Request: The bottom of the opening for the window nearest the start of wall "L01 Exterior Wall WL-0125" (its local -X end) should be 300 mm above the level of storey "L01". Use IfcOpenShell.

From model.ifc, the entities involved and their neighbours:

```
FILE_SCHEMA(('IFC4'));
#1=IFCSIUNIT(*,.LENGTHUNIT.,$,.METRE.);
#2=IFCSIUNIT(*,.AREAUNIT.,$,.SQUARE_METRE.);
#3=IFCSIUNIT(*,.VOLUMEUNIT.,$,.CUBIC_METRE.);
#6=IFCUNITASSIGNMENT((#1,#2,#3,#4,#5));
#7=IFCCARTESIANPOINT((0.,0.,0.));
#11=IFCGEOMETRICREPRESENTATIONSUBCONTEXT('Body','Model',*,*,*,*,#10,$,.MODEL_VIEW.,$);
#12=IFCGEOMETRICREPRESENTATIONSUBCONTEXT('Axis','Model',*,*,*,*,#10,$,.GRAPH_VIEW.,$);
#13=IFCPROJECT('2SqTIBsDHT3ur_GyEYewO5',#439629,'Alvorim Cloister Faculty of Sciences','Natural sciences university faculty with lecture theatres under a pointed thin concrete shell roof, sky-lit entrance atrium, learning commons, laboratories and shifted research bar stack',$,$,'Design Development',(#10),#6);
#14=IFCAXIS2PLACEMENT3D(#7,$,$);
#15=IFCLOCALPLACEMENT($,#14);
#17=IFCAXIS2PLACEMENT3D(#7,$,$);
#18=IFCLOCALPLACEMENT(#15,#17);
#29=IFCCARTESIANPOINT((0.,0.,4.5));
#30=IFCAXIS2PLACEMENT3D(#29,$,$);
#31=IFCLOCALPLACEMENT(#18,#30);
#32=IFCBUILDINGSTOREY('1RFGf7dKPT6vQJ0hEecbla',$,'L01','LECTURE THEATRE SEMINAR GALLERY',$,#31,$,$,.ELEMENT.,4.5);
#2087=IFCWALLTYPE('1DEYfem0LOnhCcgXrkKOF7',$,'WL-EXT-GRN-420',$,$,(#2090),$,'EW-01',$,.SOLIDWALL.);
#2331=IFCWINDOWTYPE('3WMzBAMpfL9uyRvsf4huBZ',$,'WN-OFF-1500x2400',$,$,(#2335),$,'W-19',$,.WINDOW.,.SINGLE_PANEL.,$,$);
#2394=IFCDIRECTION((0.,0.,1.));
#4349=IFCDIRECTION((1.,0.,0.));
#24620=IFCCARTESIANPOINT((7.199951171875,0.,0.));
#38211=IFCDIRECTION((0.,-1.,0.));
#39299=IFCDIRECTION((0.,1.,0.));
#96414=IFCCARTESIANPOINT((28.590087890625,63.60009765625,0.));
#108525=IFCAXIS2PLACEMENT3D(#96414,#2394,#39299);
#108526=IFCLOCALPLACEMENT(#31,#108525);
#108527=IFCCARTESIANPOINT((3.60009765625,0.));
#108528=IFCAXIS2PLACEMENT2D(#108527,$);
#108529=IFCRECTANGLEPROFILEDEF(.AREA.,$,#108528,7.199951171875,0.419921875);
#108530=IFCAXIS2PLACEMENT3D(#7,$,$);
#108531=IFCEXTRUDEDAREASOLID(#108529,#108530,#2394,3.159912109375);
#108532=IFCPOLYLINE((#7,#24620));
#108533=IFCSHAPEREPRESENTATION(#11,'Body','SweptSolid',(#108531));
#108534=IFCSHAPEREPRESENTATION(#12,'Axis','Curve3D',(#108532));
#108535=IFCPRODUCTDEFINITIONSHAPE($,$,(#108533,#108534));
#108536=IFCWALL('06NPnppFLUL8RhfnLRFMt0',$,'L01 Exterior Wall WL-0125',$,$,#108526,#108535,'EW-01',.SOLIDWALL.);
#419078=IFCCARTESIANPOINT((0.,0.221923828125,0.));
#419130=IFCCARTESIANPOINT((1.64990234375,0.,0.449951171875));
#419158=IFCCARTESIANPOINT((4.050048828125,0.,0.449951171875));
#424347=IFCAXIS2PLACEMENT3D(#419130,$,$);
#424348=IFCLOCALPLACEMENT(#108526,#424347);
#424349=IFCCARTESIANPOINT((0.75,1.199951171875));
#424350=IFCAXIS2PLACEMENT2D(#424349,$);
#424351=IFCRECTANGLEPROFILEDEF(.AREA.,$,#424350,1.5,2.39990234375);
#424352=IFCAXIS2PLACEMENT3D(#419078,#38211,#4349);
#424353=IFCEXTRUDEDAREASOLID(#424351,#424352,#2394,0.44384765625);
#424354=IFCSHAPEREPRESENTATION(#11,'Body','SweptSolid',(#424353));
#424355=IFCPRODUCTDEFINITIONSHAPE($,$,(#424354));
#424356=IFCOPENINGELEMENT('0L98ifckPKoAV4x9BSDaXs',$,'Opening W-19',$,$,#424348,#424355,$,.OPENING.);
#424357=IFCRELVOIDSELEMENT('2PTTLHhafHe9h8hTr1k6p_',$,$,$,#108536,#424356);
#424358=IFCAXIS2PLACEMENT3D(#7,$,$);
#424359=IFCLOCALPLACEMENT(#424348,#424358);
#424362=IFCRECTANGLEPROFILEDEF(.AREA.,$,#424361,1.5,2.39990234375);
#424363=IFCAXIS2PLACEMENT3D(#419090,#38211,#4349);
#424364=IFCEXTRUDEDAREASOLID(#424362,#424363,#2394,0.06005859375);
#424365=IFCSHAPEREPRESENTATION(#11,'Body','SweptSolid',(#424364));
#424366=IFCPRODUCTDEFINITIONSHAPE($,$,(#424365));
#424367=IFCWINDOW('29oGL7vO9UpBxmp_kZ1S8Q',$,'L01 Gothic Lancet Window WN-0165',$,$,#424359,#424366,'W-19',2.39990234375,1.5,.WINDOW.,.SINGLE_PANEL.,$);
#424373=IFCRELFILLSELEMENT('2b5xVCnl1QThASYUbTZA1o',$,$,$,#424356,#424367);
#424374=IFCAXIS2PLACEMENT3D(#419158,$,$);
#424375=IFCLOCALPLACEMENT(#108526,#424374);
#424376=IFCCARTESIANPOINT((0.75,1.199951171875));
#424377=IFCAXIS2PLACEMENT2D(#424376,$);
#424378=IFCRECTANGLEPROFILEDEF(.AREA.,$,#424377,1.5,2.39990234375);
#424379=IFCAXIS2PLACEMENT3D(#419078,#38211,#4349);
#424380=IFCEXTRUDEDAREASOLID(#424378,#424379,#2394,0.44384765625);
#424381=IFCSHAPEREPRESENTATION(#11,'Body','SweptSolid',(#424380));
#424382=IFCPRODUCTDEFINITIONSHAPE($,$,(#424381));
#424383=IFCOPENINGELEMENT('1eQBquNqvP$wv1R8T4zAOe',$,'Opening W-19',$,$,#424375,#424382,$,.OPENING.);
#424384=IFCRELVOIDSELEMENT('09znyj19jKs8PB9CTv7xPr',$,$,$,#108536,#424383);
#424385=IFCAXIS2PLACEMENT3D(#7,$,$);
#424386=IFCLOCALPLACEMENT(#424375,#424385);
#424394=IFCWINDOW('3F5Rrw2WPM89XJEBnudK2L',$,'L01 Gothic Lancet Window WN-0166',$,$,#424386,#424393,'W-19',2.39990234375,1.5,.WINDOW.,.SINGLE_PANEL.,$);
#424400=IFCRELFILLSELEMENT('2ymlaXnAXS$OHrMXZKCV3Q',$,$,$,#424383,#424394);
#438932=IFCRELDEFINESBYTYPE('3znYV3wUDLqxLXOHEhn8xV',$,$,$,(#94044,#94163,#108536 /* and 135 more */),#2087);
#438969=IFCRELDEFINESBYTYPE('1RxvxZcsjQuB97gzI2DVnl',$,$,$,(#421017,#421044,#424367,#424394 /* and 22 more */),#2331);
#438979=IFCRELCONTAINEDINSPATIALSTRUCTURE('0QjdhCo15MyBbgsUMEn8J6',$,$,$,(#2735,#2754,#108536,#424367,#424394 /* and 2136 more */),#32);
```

```python
import numpy as np
import ifcopenshell
import ifcopenshell.api.geometry
import ifcopenshell.geom
import ifcopenshell.util.element
import ifcopenshell.util.placement
import ifcopenshell.util.shape
import ifcopenshell.util.unit

model = ifcopenshell.open("model.ifc")
unit_scale = ifcopenshell.util.unit.calculate_unit_scale(model)

window = model.by_guid("29oGL7vO9UpBxmp_kZ1S8Q")
opening = window.FillsVoids[0].RelatingOpeningElement
storey = ifcopenshell.util.element.get_container(window, ifc_class="IfcBuildingStorey")
level = ifcopenshell.util.placement.get_local_placement(storey.ObjectPlacement)[2, 3]

# The opening's origin need not be at the sill, so measure its lowest point.
shape = ifcopenshell.geom.create_shape(ifcopenshell.geom.settings(), opening)
bottom = ifcopenshell.util.shape.get_shape_bottom_elevation(shape, shape.geometry) / unit_scale
dz = level + 0.3 / unit_scale - bottom

shift = np.array([0.0, 0.0, dz])
# The window is placed relative to its opening, so it follows when the opening moves.
matrix = ifcopenshell.util.placement.get_local_placement(opening.ObjectPlacement)
matrix[:3, 3] += shift
ifcopenshell.api.geometry.edit_object_placement(
    model, product=opening, matrix=matrix, is_si=False, should_transform_children=True
)

print(f"moved by {dz * unit_scale:+.3f} m")

model.write("model_updated.ifc")
```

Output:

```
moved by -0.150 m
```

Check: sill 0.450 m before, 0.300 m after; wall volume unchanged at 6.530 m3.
